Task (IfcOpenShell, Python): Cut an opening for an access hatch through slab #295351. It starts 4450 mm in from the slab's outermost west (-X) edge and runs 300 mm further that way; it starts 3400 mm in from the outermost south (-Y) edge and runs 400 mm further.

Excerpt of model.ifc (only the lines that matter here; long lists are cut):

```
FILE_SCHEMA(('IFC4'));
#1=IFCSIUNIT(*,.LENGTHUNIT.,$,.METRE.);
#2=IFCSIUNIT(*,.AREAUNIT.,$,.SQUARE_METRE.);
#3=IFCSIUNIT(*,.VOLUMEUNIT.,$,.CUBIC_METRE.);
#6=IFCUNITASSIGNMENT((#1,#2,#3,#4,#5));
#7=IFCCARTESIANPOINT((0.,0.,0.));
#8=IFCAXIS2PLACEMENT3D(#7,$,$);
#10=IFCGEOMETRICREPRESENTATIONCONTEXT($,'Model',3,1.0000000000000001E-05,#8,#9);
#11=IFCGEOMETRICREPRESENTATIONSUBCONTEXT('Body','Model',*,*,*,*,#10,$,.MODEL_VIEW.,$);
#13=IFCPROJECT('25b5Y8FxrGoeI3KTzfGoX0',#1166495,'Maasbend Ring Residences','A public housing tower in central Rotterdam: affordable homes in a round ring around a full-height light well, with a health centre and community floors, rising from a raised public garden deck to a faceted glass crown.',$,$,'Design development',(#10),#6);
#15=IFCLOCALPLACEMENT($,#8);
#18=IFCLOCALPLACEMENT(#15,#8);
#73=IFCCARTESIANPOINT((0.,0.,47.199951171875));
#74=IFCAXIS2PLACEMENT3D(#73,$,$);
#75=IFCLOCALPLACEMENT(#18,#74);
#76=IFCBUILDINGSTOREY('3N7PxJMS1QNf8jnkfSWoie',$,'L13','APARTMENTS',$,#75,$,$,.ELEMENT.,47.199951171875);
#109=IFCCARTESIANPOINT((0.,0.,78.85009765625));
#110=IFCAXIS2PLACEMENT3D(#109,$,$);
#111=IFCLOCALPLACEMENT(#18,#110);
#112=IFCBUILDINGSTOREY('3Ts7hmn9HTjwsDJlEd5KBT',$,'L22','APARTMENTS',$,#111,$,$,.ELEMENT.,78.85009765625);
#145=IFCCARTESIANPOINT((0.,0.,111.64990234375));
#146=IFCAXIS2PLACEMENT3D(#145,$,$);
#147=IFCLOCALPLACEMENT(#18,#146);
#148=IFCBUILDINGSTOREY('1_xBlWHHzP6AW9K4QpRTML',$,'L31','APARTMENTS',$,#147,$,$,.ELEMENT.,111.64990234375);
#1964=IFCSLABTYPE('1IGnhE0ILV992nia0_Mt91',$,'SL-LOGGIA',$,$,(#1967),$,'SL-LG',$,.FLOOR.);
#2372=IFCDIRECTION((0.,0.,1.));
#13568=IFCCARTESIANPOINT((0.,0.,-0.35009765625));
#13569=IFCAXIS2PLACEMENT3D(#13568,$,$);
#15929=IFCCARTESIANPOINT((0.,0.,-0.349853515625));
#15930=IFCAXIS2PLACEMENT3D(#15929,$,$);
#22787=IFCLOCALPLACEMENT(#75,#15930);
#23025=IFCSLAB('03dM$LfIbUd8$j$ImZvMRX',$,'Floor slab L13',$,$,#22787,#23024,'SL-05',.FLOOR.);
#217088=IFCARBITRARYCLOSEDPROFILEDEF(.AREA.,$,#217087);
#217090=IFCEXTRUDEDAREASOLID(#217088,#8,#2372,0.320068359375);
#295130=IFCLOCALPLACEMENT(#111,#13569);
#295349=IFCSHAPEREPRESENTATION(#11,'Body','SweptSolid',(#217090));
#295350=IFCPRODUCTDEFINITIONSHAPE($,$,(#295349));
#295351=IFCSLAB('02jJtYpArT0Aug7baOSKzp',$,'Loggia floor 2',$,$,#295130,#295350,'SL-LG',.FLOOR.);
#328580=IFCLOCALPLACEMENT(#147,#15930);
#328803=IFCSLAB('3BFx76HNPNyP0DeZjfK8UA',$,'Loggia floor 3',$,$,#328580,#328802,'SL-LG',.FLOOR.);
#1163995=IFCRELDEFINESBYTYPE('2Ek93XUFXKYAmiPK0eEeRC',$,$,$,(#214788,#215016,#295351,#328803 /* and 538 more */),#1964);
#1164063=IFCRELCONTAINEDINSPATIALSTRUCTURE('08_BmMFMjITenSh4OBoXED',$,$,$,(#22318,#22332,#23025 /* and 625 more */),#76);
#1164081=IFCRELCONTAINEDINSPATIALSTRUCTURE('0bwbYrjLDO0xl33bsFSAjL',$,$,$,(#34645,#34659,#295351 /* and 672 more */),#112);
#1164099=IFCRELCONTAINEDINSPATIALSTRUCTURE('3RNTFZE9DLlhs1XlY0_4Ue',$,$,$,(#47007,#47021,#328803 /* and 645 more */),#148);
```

```python
import numpy as np
import ifcopenshell
import ifcopenshell.api.feature
import ifcopenshell.api.geometry
import ifcopenshell.api.root
import ifcopenshell.geom
import ifcopenshell.util.placement
import ifcopenshell.util.representation
import ifcopenshell.util.shape
import ifcopenshell.util.unit

model = ifcopenshell.open("model.ifc")
unit_scale = ifcopenshell.util.unit.calculate_unit_scale(model)
settings = ifcopenshell.geom.settings()


def volume(element):
    """Net volume in cubic metres, openings subtracted."""
    shape = ifcopenshell.geom.create_shape(settings, element)
    return ifcopenshell.util.shape.get_volume(shape.geometry)


slab = model.by_guid("02jJtYpArT0Aug7baOSKzp")
before = volume(slab)

# Extent in the slab's own axes, in metres. The edges named are its -X and -Y sides.
slab_shape = ifcopenshell.geom.create_shape(settings, slab)
vertices = ifcopenshell.util.shape.get_vertices(slab_shape.geometry)
x_min, y_min, bottom = vertices.min(axis=0)
top = vertices[:, 2].max()

opening = ifcopenshell.api.root.create_entity(model, ifc_class="IfcOpeningElement", name="Access hatch opening", predefined_type="OPENING")
context = ifcopenshell.util.representation.get_context(model, "Model", "Body", "MODEL_VIEW")
width, depth = 0.3, 0.4
outline = [(0.0, 0.0), (width, 0.0), (width, depth), (0.0, depth), (0.0, 0.0)]
# Overshoot both faces by 50 mm so the cut is clean.
shape = ifcopenshell.api.geometry.add_slab_representation(
    model, context=context, depth=top - bottom + 0.1, polyline=outline
)
ifcopenshell.api.geometry.assign_representation(model, product=opening, representation=shape)

matrix = ifcopenshell.util.placement.get_local_placement(slab.ObjectPlacement)
matrix[:, 3] = matrix @ np.append(np.array([x_min + 4.45, y_min + 3.4, bottom - 0.05]) / unit_scale, 1.0)
ifcopenshell.api.geometry.edit_object_placement(model, product=opening, matrix=matrix, is_si=False)
ifcopenshell.api.feature.add_feature(model, feature=opening, element=slab)

after = volume(slab)

print(f"slab volume {before:.3f} -> {after:.3f} m3")

model.write("model_edited.ifc")
```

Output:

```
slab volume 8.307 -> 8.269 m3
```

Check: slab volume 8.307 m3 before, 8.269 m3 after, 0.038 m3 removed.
